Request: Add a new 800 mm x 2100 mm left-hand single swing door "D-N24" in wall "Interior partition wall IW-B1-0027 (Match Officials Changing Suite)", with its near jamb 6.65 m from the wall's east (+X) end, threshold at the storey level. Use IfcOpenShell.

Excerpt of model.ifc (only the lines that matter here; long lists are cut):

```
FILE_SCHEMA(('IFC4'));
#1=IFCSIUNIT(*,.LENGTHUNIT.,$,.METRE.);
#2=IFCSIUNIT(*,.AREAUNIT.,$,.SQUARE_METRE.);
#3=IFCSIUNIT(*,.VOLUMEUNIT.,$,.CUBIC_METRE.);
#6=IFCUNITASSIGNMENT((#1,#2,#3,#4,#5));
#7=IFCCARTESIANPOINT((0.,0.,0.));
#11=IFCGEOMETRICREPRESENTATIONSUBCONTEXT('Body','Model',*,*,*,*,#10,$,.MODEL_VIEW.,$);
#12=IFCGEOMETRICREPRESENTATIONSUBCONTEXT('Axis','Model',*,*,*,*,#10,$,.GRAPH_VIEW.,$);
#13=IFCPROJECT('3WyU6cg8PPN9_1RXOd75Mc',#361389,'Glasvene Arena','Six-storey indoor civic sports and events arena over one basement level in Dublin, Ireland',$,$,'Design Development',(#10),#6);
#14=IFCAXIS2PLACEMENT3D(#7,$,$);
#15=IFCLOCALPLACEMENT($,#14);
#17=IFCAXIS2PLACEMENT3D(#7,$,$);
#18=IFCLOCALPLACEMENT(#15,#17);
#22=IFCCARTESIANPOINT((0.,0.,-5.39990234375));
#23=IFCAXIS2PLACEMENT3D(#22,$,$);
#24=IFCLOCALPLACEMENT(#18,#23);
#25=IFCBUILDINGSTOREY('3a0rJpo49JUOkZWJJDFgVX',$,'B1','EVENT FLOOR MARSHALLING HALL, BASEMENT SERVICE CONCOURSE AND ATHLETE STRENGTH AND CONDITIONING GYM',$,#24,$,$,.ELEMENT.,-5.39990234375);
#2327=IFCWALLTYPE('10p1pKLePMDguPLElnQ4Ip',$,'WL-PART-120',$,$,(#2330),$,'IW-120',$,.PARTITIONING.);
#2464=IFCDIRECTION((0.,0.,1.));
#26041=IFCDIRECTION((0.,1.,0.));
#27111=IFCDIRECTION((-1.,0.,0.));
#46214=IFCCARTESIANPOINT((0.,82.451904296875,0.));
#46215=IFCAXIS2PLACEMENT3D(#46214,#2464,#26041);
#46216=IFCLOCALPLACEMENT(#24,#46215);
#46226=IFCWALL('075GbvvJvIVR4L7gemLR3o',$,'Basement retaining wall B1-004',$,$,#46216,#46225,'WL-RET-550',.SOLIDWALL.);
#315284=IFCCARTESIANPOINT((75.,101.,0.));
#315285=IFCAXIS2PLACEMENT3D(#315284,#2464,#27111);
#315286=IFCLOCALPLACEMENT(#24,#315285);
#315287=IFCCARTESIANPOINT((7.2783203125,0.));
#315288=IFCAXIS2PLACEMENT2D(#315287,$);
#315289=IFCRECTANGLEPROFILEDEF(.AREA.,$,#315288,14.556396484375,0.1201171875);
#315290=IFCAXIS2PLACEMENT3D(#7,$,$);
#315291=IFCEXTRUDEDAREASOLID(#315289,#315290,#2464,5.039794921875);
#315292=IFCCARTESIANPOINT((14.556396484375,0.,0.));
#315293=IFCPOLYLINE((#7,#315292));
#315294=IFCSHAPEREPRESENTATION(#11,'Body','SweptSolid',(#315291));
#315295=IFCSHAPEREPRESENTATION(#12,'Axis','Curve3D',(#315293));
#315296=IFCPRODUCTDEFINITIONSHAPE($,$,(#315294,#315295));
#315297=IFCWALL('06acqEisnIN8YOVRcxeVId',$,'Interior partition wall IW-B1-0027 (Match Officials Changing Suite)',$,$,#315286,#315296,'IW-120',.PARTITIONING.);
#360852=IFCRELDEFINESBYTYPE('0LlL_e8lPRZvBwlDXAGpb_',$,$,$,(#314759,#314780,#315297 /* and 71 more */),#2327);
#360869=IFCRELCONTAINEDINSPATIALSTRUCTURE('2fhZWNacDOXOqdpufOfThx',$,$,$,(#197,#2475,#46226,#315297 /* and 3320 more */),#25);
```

```python
import numpy as np
import ifcopenshell
import ifcopenshell.api.feature
import ifcopenshell.api.geometry
import ifcopenshell.api.root
import ifcopenshell.api.spatial
import ifcopenshell.geom
import ifcopenshell.util.element
import ifcopenshell.util.placement
import ifcopenshell.util.representation
import ifcopenshell.util.shape
import ifcopenshell.util.unit

model = ifcopenshell.open("model.ifc")
unit_scale = ifcopenshell.util.unit.calculate_unit_scale(model)
settings = ifcopenshell.geom.settings()


def volume(element):
    """Net volume in cubic metres, openings subtracted."""
    shape = ifcopenshell.geom.create_shape(settings, element)
    return ifcopenshell.util.shape.get_volume(shape.geometry)


wall = model.by_id(315297)
storey = ifcopenshell.util.element.get_container(wall, ifc_class="IfcBuildingStorey")
context = ifcopenshell.util.representation.get_context(model, "Model", "Body", "MODEL_VIEW")
before = volume(wall)

width, height, from_end, sill = 0.8, 2.1, 6.65, 0.0  # metres

# The wall runs along its own X axis, and the end named is its -X end.
wall_shape = ifcopenshell.geom.create_shape(settings, wall)
x, y, z = ifcopenshell.util.shape.get_vertices(wall_shape.geometry).T
start = x.min() + from_end
face, thickness = float(y.min()), float(y.max() - y.min())
wall_matrix = ifcopenshell.util.placement.get_local_placement(wall.ObjectPlacement)
level = ifcopenshell.util.placement.get_local_placement(storey.ObjectPlacement)[2, 3]


def in_wall(x, y):
    """Placement at x, y metres in the wall's axes, at sill height."""
    matrix = wall_matrix.copy()
    matrix[:, 3] = wall_matrix @ np.array([x / unit_scale, y / unit_scale, 0.0, 1.0])
    matrix[2, 3] = level + sill / unit_scale
    return matrix


# Opening: a box that overshoots both wall faces by 50 mm.
opening = ifcopenshell.api.root.create_entity(model, ifc_class="IfcOpeningElement", predefined_type="OPENING")
box = ifcopenshell.api.geometry.add_wall_representation(
    model, context=context, length=width, height=height, thickness=thickness + 0.1
)
ifcopenshell.api.geometry.assign_representation(model, product=opening, representation=box)
ifcopenshell.api.geometry.edit_object_placement(model, product=opening, matrix=in_wall(start, face - 0.05), is_si=False)
ifcopenshell.api.feature.add_feature(model, feature=opening, element=wall)

door = ifcopenshell.api.root.create_entity(model, ifc_class="IfcDoor", name="D-N24", predefined_type="DOOR")
door.OverallWidth, door.OverallHeight = width / unit_scale, height / unit_scale
door.OperationType = "SINGLE_SWING_LEFT"
body = ifcopenshell.api.geometry.add_door_representation(
    model,
    context=context,
    overall_width=door.OverallWidth,
    overall_height=door.OverallHeight,
    operation_type="SINGLE_SWING_LEFT",
    lining_properties={"LiningDepth": thickness / unit_scale, "ThresholdDepth": thickness / unit_scale},
)
ifcopenshell.api.geometry.assign_representation(model, product=door, representation=body)
ifcopenshell.api.spatial.assign_container(model, products=[door], relating_structure=storey)
ifcopenshell.api.feature.add_filling(model, opening=opening, element=door)

# The lining spans the wall, so the door starts at the wall face.
ifcopenshell.api.geometry.edit_object_placement(model, product=door, matrix=in_wall(start, face), is_si=False)

after = volume(wall)

print(f"wall volume {before:.3f} -> {after:.3f} m3")

model.write("model_edited.ifc")
```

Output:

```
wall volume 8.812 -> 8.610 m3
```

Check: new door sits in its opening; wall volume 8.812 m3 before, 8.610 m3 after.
